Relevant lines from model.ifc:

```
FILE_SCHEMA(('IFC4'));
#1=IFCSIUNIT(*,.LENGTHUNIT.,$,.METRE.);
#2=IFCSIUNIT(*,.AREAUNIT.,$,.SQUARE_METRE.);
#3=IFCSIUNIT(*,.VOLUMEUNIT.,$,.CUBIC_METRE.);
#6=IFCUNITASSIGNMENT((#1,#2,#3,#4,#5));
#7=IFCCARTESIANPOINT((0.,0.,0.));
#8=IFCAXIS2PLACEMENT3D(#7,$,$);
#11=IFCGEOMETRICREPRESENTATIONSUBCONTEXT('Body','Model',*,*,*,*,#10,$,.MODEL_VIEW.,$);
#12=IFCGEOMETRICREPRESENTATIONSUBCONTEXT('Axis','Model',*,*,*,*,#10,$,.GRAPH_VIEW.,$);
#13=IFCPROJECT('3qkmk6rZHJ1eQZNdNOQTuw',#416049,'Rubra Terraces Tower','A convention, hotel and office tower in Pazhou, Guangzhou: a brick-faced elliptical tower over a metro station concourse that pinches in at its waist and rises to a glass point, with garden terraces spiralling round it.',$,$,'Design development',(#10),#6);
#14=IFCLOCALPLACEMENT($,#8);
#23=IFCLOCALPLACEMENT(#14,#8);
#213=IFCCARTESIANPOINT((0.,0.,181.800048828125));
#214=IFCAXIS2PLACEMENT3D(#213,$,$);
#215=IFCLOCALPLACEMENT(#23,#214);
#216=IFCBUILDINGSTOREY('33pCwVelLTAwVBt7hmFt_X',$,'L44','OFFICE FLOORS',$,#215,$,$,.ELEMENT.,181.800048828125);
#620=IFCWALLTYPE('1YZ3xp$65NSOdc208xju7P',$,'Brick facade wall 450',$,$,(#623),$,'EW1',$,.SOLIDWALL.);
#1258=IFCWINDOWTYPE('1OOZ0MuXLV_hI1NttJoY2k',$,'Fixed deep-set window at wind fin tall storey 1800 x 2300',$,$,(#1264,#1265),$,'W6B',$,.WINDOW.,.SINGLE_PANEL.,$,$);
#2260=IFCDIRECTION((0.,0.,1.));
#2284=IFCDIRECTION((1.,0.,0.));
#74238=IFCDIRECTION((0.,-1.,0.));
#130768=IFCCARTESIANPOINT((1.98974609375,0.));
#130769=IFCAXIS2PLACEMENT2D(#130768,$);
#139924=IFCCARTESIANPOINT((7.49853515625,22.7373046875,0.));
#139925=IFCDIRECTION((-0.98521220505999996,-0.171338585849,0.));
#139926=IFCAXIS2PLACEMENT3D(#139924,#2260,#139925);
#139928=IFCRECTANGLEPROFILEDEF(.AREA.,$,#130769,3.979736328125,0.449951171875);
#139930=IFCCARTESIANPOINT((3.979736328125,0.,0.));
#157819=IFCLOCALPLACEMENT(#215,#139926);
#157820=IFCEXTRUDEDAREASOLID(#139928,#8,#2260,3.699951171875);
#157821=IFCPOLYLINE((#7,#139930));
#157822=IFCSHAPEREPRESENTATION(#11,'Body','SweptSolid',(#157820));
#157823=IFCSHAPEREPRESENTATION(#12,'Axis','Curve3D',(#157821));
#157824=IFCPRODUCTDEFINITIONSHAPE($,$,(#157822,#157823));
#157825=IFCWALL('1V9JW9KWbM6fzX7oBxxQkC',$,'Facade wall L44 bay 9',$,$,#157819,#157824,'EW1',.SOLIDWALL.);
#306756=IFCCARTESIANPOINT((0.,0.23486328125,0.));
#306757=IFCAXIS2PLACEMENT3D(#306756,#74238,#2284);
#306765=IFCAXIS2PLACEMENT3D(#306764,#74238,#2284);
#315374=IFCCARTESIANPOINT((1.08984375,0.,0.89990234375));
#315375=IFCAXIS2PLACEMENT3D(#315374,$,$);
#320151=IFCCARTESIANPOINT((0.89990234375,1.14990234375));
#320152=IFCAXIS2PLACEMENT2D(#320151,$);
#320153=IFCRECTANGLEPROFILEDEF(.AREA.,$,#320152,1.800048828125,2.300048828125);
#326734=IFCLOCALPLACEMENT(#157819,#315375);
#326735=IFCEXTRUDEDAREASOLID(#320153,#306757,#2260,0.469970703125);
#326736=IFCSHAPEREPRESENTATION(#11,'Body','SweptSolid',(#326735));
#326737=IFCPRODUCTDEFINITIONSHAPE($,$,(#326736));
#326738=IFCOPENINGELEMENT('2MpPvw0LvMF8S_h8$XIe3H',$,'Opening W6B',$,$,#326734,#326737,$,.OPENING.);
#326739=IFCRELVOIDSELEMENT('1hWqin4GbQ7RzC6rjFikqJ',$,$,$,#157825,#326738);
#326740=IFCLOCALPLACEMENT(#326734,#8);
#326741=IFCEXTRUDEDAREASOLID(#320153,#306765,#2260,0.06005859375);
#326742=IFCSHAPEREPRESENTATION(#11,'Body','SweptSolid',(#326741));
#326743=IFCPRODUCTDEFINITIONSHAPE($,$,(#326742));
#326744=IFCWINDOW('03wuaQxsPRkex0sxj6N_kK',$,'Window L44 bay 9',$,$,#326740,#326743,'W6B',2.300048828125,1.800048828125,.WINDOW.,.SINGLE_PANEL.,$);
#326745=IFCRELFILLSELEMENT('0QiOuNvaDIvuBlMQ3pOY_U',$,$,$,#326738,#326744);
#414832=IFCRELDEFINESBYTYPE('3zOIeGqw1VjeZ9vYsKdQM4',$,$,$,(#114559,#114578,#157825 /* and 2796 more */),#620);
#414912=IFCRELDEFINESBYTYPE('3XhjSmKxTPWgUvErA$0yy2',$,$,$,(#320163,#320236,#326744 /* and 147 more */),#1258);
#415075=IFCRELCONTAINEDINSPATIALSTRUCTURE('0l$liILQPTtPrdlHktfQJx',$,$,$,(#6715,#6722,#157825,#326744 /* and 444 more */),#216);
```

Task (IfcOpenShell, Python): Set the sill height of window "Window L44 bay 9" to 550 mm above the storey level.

```python
import numpy as np
import ifcopenshell
import ifcopenshell.api.geometry
import ifcopenshell.geom
import ifcopenshell.util.element
import ifcopenshell.util.placement
import ifcopenshell.util.shape
import ifcopenshell.util.unit

model = ifcopenshell.open("model.ifc")
unit_scale = ifcopenshell.util.unit.calculate_unit_scale(model)

window = model.by_guid("03wuaQxsPRkex0sxj6N_kK")
opening = window.FillsVoids[0].RelatingOpeningElement
storey = ifcopenshell.util.element.get_container(window, ifc_class="IfcBuildingStorey")
level = ifcopenshell.util.placement.get_local_placement(storey.ObjectPlacement)[2, 3]

# The opening's origin need not be at the sill, so measure its lowest point.
shape = ifcopenshell.geom.create_shape(ifcopenshell.geom.settings(), opening)
bottom = ifcopenshell.util.shape.get_shape_bottom_elevation(shape, shape.geometry) / unit_scale
dz = level + 0.55 - bottom

shift = np.array([0.0, 0.0, dz])
# The window is placed relative to its opening, so it follows when the opening moves.
matrix = ifcopenshell.util.placement.get_local_placement(opening.ObjectPlacement)
matrix[:3, 3] += shift
ifcopenshell.api.geometry.edit_object_placement(
    model, product=opening, matrix=matrix, is_si=False, should_transform_children=True
)

print(f"moved by {dz * unit_scale:+.3f} m")

model.write("model_v2.ifc")
```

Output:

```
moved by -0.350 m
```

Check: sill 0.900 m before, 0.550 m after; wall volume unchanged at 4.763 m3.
